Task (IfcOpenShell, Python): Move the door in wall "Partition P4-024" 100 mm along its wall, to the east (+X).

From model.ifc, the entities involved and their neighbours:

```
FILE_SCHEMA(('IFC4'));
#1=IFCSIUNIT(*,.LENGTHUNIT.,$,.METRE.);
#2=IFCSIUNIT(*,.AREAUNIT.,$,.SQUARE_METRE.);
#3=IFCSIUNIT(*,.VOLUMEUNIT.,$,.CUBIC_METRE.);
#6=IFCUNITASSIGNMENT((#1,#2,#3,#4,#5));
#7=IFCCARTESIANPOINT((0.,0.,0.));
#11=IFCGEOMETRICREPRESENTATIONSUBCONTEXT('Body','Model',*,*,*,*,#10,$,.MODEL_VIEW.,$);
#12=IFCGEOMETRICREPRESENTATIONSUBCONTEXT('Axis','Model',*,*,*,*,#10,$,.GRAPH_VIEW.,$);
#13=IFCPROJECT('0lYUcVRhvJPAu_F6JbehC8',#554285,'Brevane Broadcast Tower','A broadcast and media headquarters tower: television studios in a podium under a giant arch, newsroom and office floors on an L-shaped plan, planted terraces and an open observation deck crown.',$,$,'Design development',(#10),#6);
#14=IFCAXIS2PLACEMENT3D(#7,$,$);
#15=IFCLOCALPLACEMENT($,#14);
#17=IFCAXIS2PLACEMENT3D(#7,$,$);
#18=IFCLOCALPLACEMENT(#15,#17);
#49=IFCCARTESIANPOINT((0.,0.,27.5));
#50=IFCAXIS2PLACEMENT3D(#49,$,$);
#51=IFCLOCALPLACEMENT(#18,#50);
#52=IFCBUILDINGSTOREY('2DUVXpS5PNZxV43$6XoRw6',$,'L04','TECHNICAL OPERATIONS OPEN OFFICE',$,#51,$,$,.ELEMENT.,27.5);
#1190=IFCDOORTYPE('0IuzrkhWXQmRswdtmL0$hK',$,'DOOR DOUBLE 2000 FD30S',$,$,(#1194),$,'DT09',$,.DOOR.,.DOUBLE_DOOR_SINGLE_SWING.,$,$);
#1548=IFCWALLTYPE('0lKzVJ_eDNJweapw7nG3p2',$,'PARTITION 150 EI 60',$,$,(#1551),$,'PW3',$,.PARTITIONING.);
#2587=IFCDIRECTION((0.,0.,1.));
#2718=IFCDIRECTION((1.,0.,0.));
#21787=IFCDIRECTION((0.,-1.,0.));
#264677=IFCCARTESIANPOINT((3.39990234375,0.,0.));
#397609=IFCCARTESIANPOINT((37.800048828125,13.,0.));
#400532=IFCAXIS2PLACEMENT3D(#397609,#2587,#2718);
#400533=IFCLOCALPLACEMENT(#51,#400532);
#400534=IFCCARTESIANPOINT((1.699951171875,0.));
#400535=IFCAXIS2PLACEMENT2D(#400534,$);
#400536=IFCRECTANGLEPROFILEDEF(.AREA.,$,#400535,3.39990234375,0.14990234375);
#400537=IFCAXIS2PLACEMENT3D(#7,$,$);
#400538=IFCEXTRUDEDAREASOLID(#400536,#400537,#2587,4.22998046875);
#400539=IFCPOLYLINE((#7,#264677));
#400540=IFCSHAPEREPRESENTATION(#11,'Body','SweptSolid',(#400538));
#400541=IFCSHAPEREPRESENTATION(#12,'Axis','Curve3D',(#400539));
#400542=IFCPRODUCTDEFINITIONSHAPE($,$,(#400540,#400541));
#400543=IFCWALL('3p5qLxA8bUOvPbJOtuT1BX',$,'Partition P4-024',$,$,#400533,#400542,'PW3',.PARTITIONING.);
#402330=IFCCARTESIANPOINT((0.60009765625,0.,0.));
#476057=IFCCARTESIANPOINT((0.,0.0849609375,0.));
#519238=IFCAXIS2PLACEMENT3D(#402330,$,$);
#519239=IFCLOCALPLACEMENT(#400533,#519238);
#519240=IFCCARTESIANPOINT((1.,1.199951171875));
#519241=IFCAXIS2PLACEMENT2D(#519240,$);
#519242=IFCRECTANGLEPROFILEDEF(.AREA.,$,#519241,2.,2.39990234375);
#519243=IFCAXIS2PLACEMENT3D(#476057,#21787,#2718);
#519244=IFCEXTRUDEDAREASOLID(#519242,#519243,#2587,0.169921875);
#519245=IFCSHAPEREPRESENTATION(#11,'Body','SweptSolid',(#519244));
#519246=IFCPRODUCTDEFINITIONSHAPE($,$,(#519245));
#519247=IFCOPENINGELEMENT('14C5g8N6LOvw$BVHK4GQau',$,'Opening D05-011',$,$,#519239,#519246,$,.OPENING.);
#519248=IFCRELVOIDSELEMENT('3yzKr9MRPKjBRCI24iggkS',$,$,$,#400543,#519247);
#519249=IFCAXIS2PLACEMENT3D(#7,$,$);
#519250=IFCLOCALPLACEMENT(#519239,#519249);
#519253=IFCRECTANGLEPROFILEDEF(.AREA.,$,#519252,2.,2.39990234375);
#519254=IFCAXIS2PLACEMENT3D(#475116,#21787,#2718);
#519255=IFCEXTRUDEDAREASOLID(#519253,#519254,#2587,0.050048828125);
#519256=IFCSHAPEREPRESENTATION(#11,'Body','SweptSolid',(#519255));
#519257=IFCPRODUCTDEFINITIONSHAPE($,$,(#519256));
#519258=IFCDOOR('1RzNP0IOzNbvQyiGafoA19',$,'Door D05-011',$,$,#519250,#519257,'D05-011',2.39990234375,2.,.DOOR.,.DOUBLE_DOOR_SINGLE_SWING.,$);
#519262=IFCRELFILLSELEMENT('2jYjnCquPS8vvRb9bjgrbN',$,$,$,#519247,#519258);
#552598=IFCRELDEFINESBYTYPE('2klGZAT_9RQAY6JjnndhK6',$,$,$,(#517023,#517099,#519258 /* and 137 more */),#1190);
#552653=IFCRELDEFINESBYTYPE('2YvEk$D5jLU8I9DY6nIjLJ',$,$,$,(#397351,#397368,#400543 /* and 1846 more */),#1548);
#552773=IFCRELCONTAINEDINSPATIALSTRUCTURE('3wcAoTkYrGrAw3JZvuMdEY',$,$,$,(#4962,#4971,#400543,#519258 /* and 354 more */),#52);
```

```python
import ifcopenshell
import ifcopenshell.api.geometry
import ifcopenshell.util.placement

model = ifcopenshell.open("model.ifc")

door = model.by_guid("1RzNP0IOzNbvQyiGafoA19")
opening = door.FillsVoids[0].RelatingOpeningElement
wall = opening.VoidsElements[0].RelatingBuildingElement

wall_matrix = ifcopenshell.util.placement.get_local_placement(wall.ObjectPlacement)
shift = wall_matrix[:3, 0] * 0.1
before = ifcopenshell.util.placement.get_local_placement(door.ObjectPlacement)[:3, 3].copy()

# The door is placed relative to its opening, so it follows when the opening moves.
matrix = ifcopenshell.util.placement.get_local_placement(opening.ObjectPlacement)
matrix[:3, 3] += shift
ifcopenshell.api.geometry.edit_object_placement(
    model, product=opening, matrix=matrix, is_si=False, should_transform_children=True
)

after = ifcopenshell.util.placement.get_local_placement(door.ObjectPlacement)[:3, 3]
print("door moved by", (after - before).round(3) + 0.0)

model.write("model_edited.ifc")
```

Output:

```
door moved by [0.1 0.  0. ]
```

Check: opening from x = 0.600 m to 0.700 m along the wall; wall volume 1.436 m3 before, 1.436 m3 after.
